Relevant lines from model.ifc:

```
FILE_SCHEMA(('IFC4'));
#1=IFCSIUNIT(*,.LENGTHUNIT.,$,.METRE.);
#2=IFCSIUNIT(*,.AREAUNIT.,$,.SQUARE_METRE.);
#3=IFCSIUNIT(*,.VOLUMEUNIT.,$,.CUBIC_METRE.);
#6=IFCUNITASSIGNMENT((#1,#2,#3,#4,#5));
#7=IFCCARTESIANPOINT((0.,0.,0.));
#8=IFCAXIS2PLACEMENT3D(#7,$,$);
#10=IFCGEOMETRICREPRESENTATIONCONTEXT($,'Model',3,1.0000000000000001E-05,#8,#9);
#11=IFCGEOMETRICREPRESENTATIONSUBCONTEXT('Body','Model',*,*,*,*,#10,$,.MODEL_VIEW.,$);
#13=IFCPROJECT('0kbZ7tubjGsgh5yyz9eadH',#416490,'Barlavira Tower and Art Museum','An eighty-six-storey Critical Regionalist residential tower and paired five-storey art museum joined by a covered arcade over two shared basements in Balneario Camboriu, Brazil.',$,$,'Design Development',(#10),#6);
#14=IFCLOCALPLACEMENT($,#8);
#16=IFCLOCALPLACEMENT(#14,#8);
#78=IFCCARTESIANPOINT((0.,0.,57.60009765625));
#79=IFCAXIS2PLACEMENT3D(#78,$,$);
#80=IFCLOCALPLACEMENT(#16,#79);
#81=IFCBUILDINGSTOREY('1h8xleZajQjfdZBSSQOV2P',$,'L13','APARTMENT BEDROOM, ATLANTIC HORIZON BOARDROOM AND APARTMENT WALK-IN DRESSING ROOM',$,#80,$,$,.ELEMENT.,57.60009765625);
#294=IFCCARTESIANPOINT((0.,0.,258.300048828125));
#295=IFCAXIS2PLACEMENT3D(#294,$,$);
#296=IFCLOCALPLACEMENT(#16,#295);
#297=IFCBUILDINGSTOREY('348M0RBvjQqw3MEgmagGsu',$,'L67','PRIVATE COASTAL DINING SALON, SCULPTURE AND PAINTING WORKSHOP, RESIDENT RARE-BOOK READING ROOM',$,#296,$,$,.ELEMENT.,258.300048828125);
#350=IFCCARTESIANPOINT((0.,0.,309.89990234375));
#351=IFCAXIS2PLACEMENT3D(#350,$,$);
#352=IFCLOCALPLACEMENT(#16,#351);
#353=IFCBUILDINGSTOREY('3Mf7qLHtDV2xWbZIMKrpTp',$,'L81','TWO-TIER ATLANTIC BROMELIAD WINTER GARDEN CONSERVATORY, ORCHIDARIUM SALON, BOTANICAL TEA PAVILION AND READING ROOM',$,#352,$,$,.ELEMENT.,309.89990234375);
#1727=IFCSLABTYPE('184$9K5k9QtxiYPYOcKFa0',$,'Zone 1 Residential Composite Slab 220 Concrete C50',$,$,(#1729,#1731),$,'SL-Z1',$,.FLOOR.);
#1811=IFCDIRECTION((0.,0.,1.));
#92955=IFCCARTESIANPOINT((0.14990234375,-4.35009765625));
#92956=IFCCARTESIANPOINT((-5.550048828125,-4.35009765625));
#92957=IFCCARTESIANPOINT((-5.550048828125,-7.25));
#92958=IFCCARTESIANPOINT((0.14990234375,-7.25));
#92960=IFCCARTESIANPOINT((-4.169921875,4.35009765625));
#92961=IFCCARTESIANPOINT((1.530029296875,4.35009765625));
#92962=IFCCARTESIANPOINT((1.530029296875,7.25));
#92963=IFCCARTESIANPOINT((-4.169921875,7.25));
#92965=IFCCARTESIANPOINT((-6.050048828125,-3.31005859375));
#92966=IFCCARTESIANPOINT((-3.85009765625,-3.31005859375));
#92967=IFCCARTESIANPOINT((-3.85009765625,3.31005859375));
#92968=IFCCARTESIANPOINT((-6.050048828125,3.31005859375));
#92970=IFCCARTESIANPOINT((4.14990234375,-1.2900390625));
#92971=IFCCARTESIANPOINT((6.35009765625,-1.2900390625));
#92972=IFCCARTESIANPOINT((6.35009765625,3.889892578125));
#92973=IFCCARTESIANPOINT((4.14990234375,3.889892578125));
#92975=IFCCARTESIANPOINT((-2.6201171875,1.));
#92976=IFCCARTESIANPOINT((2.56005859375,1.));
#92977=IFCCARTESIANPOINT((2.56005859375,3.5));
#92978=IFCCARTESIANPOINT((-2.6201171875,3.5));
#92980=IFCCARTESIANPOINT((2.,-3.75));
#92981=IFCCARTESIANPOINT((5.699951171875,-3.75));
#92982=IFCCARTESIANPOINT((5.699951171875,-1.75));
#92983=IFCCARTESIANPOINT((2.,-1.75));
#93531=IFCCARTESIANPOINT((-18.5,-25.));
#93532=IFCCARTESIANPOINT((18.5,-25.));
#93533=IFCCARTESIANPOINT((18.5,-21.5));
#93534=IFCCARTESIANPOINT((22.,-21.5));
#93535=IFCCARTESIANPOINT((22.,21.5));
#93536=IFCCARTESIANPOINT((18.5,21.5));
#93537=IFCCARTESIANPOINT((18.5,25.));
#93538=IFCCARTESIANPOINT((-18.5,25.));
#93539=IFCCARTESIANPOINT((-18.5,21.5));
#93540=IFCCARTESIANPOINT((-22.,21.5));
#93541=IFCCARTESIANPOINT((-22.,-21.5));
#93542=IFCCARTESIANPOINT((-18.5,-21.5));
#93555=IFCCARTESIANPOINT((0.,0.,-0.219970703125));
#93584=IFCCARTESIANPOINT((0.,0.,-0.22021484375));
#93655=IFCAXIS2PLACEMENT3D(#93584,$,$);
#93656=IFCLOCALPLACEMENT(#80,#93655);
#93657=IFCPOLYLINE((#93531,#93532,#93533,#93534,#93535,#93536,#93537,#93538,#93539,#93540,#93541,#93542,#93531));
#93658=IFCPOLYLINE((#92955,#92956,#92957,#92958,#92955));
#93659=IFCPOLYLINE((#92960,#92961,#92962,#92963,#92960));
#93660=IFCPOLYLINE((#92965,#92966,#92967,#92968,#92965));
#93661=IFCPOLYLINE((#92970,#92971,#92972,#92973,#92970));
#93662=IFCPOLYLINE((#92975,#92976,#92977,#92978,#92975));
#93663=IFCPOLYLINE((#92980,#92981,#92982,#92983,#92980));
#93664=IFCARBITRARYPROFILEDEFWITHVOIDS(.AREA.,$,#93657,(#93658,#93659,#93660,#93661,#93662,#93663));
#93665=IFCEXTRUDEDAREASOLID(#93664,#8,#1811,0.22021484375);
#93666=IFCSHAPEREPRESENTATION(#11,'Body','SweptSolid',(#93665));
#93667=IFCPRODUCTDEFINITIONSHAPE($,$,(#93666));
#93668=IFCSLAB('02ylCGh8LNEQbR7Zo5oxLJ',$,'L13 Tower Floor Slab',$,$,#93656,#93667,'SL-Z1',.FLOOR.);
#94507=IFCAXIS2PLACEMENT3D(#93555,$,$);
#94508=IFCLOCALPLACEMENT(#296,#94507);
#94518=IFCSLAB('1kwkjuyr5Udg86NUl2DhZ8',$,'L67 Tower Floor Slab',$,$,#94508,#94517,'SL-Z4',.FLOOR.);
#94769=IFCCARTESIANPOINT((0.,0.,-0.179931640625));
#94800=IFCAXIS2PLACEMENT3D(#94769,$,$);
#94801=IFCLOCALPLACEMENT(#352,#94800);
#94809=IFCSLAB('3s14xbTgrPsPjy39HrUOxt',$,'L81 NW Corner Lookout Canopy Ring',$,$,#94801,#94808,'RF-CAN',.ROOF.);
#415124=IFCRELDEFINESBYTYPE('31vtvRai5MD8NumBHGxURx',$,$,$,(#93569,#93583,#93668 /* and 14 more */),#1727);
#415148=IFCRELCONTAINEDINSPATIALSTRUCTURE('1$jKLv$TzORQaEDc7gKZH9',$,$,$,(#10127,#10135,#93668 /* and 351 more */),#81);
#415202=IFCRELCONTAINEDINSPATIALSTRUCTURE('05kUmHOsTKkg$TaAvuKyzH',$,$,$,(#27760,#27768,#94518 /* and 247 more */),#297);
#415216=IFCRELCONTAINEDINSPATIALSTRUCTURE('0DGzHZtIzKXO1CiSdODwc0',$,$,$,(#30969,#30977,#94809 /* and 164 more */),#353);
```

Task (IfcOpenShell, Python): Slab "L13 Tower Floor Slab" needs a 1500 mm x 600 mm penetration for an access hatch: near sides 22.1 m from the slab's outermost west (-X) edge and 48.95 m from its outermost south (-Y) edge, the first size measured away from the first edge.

```python
import numpy as np
import ifcopenshell
import ifcopenshell.api.feature
import ifcopenshell.api.geometry
import ifcopenshell.api.root
import ifcopenshell.geom
import ifcopenshell.util.placement
import ifcopenshell.util.representation
import ifcopenshell.util.shape
import ifcopenshell.util.unit

model = ifcopenshell.open("model.ifc")
unit_scale = ifcopenshell.util.unit.calculate_unit_scale(model)
settings = ifcopenshell.geom.settings()


def volume(element):
    """Net volume in cubic metres, openings subtracted."""
    shape = ifcopenshell.geom.create_shape(settings, element)
    return ifcopenshell.util.shape.get_volume(shape.geometry)


slab = model.by_guid("02ylCGh8LNEQbR7Zo5oxLJ")
before = volume(slab)

# Extent in the slab's own axes, in metres. The edges named are its -X and -Y sides.
slab_shape = ifcopenshell.geom.create_shape(settings, slab)
vertices = ifcopenshell.util.shape.get_vertices(slab_shape.geometry)
x_min, y_min, bottom = vertices.min(axis=0)
top = vertices[:, 2].max()

opening = ifcopenshell.api.root.create_entity(model, ifc_class="IfcOpeningElement", name="Access hatch opening", predefined_type="OPENING")
context = ifcopenshell.util.representation.get_context(model, "Model", "Body", "MODEL_VIEW")
width, depth = 1.5, 0.6
outline = [(0.0, 0.0), (width, 0.0), (width, depth), (0.0, depth), (0.0, 0.0)]
# Overshoot both faces by 50 mm so the cut is clean.
shape = ifcopenshell.api.geometry.add_slab_representation(
    model, context=context, depth=top - bottom + 0.1, polyline=outline
)
ifcopenshell.api.geometry.assign_representation(model, product=opening, representation=shape)

matrix = ifcopenshell.util.placement.get_local_placement(slab.ObjectPlacement)
matrix[:, 3] = matrix @ np.append(np.array([x_min + 22.1, y_min + 48.95, bottom - 0.05]) / unit_scale, 1.0)
ifcopenshell.api.geometry.edit_object_placement(model, product=opening, matrix=matrix, is_si=False)
ifcopenshell.api.feature.add_feature(model, feature=opening, element=slab)

after = volume(slab)

print(f"slab volume {before:.3f} -> {after:.3f} m3")

model.write("model_rev.ifc")
```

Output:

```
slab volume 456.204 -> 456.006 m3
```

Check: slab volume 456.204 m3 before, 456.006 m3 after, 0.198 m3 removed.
